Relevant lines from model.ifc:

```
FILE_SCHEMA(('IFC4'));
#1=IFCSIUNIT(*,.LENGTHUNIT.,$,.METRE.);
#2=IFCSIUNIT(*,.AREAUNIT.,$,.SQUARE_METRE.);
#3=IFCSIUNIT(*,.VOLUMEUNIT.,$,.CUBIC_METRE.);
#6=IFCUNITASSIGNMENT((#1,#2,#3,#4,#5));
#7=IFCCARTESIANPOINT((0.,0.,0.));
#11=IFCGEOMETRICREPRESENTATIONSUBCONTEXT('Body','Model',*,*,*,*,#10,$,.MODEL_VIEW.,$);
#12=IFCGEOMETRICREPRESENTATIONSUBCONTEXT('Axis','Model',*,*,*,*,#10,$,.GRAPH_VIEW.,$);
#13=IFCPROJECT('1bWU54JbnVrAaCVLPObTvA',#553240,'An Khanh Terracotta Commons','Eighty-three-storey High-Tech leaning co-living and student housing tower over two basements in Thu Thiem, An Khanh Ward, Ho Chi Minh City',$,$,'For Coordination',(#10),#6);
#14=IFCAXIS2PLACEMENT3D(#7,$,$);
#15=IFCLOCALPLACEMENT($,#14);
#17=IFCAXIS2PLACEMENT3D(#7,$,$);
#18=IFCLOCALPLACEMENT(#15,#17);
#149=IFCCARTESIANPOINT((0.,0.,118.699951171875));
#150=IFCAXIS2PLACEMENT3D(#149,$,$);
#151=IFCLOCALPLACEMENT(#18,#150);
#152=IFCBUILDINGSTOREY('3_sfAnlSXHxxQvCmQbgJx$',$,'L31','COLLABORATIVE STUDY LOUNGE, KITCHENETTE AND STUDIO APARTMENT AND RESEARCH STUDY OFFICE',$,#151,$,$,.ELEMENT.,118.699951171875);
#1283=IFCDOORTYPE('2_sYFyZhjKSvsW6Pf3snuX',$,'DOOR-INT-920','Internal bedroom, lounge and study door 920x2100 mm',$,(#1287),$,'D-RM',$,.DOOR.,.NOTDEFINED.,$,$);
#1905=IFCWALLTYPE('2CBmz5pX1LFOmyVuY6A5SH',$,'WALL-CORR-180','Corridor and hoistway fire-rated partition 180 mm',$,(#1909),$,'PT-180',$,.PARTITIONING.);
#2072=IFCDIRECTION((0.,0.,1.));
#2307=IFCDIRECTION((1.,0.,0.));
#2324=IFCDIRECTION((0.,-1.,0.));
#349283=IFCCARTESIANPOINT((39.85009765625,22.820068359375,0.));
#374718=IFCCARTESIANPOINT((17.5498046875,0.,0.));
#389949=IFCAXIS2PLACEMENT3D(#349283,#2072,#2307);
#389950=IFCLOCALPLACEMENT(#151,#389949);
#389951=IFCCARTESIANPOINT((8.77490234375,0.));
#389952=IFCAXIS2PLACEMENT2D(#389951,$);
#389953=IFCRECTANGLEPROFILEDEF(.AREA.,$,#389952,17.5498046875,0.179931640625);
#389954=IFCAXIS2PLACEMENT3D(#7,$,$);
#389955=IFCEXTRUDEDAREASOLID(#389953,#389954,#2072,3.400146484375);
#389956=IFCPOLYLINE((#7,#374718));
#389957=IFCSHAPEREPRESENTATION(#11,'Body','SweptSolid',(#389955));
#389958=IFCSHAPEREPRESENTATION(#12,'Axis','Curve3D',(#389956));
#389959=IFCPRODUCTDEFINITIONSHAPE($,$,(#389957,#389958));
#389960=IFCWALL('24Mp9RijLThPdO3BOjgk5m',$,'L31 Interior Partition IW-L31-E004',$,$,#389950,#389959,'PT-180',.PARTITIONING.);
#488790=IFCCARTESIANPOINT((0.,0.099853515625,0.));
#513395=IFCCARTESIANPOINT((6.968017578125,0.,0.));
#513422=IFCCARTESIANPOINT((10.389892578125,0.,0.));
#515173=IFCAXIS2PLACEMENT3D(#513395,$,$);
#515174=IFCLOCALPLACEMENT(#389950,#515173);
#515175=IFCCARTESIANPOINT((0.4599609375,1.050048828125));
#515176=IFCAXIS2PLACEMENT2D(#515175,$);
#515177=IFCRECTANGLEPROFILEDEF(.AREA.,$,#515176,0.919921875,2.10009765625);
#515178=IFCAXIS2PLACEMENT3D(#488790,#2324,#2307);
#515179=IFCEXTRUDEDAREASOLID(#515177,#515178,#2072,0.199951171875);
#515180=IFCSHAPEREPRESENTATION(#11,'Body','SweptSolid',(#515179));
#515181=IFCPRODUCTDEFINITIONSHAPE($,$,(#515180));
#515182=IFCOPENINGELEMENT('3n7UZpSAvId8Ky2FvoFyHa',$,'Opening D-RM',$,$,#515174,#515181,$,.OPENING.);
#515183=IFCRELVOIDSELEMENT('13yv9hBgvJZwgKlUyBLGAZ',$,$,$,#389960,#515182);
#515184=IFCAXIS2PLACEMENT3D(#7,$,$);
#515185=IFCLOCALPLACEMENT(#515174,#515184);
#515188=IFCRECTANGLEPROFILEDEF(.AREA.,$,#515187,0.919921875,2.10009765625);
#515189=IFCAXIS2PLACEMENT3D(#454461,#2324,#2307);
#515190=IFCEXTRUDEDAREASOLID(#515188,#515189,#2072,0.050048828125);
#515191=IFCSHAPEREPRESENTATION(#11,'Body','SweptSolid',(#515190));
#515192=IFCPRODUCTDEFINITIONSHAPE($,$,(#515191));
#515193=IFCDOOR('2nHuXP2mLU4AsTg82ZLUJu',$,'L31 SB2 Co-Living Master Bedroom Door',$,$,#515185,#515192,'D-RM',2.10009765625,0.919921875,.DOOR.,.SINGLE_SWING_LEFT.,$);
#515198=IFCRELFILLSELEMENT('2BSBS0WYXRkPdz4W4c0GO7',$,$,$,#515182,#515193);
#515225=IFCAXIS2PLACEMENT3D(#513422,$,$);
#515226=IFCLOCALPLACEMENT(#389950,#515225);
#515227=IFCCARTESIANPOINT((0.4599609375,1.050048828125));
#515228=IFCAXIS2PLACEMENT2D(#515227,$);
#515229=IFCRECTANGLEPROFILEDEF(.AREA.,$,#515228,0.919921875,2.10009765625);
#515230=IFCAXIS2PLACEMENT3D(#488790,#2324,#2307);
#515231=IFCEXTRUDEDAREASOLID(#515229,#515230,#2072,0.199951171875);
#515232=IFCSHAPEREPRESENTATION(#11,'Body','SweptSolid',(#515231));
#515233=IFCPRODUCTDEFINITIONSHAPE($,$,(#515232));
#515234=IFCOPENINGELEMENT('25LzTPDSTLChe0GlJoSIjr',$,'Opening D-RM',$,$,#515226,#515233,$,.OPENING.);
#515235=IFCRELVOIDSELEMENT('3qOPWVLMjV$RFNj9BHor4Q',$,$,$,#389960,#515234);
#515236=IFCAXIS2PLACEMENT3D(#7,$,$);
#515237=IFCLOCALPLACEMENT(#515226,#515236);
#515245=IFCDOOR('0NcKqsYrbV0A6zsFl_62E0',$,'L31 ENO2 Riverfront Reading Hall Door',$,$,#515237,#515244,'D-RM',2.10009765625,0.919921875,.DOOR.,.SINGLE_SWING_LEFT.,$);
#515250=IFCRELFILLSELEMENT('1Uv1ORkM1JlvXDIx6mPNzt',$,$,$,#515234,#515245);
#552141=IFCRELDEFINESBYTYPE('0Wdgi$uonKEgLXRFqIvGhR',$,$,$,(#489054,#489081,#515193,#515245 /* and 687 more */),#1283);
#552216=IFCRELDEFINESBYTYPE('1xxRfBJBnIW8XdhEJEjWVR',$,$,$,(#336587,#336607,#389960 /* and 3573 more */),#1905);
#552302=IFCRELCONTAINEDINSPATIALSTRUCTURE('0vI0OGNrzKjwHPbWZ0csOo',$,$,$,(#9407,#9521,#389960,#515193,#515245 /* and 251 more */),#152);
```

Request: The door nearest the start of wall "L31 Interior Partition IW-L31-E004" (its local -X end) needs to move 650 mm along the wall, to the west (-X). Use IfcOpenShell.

```python
import ifcopenshell
import ifcopenshell.api.geometry
import ifcopenshell.util.placement
import ifcopenshell.util.unit

model = ifcopenshell.open("model.ifc")
unit_scale = ifcopenshell.util.unit.calculate_unit_scale(model)

door = model.by_id(515193)
opening = door.FillsVoids[0].RelatingOpeningElement
wall = opening.VoidsElements[0].RelatingBuildingElement

wall_matrix = ifcopenshell.util.placement.get_local_placement(wall.ObjectPlacement)
shift = wall_matrix[:3, 0] * -0.65 / unit_scale
before = ifcopenshell.util.placement.get_local_placement(door.ObjectPlacement)[:3, 3].copy()

# The door is placed relative to its opening, so it follows when the opening moves.
matrix = ifcopenshell.util.placement.get_local_placement(opening.ObjectPlacement)
matrix[:3, 3] += shift
ifcopenshell.api.geometry.edit_object_placement(
    model, product=opening, matrix=matrix, is_si=False, should_transform_children=True
)

after = ifcopenshell.util.placement.get_local_placement(door.ObjectPlacement)[:3, 3]
print("door moved by", (after - before).round(3) + 0.0)

model.write("model_updated.ifc")
```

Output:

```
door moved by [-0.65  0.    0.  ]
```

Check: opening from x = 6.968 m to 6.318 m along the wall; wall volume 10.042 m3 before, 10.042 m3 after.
